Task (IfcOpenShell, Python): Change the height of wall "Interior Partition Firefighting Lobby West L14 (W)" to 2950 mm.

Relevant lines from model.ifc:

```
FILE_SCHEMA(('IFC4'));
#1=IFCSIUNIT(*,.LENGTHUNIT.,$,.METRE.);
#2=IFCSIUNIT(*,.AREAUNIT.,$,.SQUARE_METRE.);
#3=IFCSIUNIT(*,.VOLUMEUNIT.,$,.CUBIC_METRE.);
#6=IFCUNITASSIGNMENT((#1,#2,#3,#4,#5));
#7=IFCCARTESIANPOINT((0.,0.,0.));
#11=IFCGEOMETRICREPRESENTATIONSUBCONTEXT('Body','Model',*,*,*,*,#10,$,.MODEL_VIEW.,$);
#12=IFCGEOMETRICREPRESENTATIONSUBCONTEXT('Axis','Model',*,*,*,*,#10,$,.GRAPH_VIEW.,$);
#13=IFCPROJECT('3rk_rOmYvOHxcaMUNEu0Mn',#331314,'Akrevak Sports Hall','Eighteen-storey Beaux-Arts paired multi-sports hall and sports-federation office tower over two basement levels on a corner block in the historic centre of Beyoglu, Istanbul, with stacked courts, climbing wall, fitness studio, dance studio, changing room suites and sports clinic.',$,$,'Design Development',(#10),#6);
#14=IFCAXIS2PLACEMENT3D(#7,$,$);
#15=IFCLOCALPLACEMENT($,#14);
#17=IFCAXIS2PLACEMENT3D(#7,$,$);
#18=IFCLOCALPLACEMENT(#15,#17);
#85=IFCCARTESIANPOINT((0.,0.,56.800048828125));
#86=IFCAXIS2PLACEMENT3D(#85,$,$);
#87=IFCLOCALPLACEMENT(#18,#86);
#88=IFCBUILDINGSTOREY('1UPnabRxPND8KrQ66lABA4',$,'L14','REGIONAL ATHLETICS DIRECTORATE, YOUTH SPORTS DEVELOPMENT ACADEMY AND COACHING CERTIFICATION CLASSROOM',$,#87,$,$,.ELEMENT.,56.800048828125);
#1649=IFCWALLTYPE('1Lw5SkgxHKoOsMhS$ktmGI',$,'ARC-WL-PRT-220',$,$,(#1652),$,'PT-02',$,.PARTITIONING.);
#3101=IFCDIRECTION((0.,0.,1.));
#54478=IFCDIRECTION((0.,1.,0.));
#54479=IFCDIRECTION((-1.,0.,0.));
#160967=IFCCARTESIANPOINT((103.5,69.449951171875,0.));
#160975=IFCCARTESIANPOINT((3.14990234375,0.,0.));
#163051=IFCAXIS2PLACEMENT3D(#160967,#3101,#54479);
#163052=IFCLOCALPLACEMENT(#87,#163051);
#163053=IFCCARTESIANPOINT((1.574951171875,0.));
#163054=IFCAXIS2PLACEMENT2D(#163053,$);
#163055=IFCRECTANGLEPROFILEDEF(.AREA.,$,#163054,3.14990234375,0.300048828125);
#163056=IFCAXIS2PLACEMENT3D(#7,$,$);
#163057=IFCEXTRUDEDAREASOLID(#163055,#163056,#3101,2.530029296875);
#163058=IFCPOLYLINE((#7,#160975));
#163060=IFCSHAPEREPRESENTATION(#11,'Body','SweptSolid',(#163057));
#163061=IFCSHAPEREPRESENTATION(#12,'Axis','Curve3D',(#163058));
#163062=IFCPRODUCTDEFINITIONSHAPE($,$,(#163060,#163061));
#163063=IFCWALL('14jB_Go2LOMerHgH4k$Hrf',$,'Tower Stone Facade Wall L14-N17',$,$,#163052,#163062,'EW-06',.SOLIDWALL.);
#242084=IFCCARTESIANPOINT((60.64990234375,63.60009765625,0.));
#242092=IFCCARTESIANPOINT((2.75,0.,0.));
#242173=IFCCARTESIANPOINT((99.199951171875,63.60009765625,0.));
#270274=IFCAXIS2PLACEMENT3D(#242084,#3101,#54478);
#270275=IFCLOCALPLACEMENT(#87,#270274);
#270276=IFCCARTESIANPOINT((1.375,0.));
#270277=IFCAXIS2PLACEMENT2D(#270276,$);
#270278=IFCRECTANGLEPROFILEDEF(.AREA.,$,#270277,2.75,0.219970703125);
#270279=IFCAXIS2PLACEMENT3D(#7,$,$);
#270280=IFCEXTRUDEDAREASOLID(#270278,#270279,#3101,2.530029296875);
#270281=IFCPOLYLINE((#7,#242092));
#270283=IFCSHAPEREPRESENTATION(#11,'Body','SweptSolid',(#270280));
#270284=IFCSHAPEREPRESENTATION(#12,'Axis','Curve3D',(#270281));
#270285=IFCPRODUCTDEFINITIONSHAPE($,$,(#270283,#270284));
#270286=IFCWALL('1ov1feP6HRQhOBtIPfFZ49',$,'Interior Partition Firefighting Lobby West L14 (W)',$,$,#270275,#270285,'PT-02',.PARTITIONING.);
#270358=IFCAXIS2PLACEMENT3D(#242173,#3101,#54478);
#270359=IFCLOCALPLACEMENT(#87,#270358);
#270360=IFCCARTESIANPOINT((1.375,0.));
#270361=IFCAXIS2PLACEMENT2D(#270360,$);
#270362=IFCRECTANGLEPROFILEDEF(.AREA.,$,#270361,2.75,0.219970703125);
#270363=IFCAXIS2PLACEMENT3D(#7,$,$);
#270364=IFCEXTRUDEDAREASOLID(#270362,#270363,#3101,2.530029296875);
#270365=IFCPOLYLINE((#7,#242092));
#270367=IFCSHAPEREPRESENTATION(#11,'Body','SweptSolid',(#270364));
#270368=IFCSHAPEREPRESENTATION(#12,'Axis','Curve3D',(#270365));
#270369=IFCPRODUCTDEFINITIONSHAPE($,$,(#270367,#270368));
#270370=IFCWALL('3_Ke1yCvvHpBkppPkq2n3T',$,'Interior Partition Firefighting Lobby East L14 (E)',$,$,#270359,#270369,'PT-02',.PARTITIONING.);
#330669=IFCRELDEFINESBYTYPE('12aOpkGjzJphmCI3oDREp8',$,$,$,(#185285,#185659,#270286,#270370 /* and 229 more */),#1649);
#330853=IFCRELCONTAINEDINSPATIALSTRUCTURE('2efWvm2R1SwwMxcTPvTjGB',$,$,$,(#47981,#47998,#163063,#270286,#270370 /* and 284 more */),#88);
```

```python
import ifcopenshell
import ifcopenshell.geom
import ifcopenshell.util.representation
import ifcopenshell.util.shape
import ifcopenshell.util.unit

model = ifcopenshell.open("model.ifc")
unit_scale = ifcopenshell.util.unit.calculate_unit_scale(model)
settings = ifcopenshell.geom.settings()


def volume(element):
    """Net volume in cubic metres, openings subtracted."""
    shape = ifcopenshell.geom.create_shape(settings, element)
    return ifcopenshell.util.shape.get_volume(shape.geometry)


wall = model.by_guid("1ov1feP6HRQhOBtIPfFZ49")
before = volume(wall)

body = ifcopenshell.util.representation.get_representation(wall, "Model", "Body")
solid = body.Items[0]
old_height = solid.Depth
solid.Depth = 2.95 / unit_scale
after = volume(wall)

print(f"height {old_height:g} -> {solid.Depth:g}, volume {before:.3f} -> {after:.3f} m3")

model.write("model_updated.ifc")
```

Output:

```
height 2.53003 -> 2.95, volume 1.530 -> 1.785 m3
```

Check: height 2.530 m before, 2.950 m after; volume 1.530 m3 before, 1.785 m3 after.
